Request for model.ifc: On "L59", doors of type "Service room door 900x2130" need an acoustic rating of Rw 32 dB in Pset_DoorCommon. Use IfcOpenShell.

First a look at what the model holds.

```python
import ifcopenshell
import ifcopenshell.util.element

model = ifcopenshell.open("model.ifc")
print(model.schema)
storey = next(s for s in model.by_type("IfcBuildingStorey") if s.Name == "L59")
doors = [e for e in ifcopenshell.util.element.get_decomposition(storey) if e.is_a("IfcDoor")]
seen = {}
for e in doors:
    element_type = ifcopenshell.util.element.get_type(e)
    key = (element_type.Name if element_type != e and element_type else None, ifcopenshell.util.element.get_pset(e, "Pset_DoorCommon", "AcousticRating"))
    seen[key] = seen.get(key, 0) + 1
for (name, value), count in sorted(seen.items(), key=str):
    print(count, "x", name, "|", value)
```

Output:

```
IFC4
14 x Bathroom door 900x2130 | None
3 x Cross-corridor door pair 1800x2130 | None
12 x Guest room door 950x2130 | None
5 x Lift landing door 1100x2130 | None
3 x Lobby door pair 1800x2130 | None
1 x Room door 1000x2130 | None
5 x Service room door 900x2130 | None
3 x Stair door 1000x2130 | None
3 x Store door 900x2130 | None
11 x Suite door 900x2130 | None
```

```python
import ifcopenshell
import ifcopenshell.api.pset
import ifcopenshell.util.element

model = ifcopenshell.open("model.ifc")

storey = next(s for s in model.by_type("IfcBuildingStorey") if s.Name == "L59")
doors = [e for e in ifcopenshell.util.element.get_decomposition(storey) if e.is_a("IfcDoor")]

count = 0
for e in doors:
    element_type = ifcopenshell.util.element.get_type(e)
    if element_type in (None, e) or element_type.Name != "Service room door 900x2130":
        continue
    found = ifcopenshell.util.element.get_pset(e, "Pset_DoorCommon", should_inherit=False)
    if found:
        pset = model.by_id(found["id"])
        if len(ifcopenshell.util.element.get_elements_by_pset(pset)) > 1:
            pset = ifcopenshell.api.pset.unshare_pset(model, products=[e], pset=pset)[0]
    else:
        pset = ifcopenshell.api.pset.add_pset(model, product=e, name="Pset_DoorCommon")
    ifcopenshell.api.pset.edit_pset(model, pset=pset, properties={"AcousticRating": "Rw 32 dB"})
    count += 1

print(count, "doors updated")

model.write("model_updated.ifc")
```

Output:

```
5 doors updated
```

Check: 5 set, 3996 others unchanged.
